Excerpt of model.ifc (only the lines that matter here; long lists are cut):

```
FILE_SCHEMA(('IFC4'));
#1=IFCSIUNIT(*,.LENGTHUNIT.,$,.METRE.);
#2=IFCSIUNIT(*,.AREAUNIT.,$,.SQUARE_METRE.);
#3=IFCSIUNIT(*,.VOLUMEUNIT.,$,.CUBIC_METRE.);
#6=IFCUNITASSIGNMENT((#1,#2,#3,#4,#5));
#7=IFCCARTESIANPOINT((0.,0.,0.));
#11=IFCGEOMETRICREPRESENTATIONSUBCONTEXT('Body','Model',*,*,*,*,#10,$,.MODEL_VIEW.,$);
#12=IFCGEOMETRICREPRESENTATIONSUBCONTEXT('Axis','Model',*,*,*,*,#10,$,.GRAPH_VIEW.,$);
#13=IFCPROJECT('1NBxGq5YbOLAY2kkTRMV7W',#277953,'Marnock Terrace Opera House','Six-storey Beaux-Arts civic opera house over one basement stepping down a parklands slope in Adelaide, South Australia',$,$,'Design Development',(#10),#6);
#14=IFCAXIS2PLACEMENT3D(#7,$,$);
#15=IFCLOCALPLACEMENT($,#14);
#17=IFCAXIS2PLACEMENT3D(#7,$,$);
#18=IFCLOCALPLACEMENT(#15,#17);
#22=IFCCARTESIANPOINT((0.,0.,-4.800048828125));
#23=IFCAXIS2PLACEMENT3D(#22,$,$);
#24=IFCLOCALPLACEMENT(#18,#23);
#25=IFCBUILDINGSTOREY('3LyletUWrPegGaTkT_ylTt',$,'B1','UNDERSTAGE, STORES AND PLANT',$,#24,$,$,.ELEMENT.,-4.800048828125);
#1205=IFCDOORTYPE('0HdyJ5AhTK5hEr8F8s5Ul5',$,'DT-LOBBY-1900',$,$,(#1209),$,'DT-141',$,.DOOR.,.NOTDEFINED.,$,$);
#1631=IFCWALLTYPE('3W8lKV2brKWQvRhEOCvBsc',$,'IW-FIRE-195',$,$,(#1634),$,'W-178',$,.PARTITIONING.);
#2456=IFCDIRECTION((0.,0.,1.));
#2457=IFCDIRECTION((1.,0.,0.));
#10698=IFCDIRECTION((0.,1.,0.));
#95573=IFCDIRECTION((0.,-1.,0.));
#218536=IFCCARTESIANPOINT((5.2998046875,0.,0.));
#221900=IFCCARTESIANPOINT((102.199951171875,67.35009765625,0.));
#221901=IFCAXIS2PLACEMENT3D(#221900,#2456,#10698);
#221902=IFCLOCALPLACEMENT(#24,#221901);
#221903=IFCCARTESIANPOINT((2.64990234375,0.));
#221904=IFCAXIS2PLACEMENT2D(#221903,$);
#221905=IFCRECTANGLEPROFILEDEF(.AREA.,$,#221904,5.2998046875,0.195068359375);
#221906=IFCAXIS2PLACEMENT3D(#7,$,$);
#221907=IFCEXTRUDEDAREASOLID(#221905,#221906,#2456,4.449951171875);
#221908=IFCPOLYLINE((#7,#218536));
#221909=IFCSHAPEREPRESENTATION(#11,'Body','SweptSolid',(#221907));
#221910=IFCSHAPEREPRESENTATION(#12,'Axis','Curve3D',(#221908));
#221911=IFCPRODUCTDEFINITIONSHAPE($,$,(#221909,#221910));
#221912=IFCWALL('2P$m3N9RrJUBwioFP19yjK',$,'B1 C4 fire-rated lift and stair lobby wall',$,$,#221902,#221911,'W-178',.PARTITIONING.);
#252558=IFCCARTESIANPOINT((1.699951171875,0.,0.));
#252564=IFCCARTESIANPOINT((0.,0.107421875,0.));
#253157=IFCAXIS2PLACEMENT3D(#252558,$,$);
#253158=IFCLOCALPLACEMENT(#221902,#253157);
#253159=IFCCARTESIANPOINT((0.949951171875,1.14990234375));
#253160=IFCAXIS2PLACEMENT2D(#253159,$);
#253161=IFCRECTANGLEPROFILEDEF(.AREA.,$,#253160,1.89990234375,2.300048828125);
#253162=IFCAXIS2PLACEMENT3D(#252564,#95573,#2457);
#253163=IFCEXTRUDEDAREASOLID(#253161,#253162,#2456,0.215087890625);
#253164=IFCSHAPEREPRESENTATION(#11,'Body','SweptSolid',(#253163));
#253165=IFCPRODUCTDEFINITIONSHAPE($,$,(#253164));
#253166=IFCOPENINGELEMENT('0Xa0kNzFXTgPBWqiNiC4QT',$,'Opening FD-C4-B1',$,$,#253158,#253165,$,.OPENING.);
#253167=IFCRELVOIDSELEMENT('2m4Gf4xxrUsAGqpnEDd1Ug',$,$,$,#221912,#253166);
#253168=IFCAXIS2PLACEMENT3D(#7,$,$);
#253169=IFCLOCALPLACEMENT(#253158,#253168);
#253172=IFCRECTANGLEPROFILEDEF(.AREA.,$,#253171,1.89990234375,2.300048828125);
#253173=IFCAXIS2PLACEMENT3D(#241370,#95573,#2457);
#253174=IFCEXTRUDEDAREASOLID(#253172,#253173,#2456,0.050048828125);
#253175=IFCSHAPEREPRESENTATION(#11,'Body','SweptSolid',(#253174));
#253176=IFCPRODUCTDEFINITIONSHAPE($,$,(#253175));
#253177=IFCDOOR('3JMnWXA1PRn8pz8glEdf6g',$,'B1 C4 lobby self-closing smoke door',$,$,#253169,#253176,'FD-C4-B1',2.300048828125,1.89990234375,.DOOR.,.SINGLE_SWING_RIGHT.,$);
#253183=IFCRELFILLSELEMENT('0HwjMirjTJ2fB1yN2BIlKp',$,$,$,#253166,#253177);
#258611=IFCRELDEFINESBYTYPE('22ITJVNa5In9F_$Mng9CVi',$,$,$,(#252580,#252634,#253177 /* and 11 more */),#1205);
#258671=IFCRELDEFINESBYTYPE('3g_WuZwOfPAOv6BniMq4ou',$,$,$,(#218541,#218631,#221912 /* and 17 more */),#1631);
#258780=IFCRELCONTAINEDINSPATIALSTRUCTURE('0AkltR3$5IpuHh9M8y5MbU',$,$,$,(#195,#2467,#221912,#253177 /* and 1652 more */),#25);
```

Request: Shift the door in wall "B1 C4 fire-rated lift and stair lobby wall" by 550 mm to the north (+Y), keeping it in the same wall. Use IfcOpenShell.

```python
import ifcopenshell
import ifcopenshell.api.geometry
import ifcopenshell.util.placement

model = ifcopenshell.open("model.ifc")

door = model.by_guid("3JMnWXA1PRn8pz8glEdf6g")
opening = door.FillsVoids[0].RelatingOpeningElement
wall = opening.VoidsElements[0].RelatingBuildingElement

wall_matrix = ifcopenshell.util.placement.get_local_placement(wall.ObjectPlacement)
shift = wall_matrix[:3, 0] * 0.55
before = ifcopenshell.util.placement.get_local_placement(door.ObjectPlacement)[:3, 3].copy()

# The door is placed relative to its opening, so it follows when the opening moves.
matrix = ifcopenshell.util.placement.get_local_placement(opening.ObjectPlacement)
matrix[:3, 3] += shift
ifcopenshell.api.geometry.edit_object_placement(
    model, product=opening, matrix=matrix, is_si=False, should_transform_children=True
)

after = ifcopenshell.util.placement.get_local_placement(door.ObjectPlacement)[:3, 3]
print("door moved by", (after - before).round(3) + 0.0)

model.write("model_rev.ifc")
```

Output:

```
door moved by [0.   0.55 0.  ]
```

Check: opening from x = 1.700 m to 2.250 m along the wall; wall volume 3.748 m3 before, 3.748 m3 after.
